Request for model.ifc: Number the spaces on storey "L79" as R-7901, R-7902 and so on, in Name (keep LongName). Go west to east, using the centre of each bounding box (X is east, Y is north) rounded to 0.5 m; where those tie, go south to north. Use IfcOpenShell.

First a look at what the model holds.

```python
import ifcopenshell
import ifcopenshell.util.element
import ifcopenshell.util.placement

model = ifcopenshell.open("model.ifc")
print(model.schema)
storey = next(s for s in model.by_type("IfcBuildingStorey") if s.Name == "L79")
spaces = [e for e in ifcopenshell.util.element.get_decomposition(storey) if e.is_a("IfcSpace")]
for e in sorted(spaces, key=lambda e: e.id()):
    origin = ifcopenshell.util.placement.get_local_placement(e.ObjectPlacement)[:3, 3]
    print(e.id(), e.Name, e.LongName, origin.round(2) + 0.0, sep=" | ")
```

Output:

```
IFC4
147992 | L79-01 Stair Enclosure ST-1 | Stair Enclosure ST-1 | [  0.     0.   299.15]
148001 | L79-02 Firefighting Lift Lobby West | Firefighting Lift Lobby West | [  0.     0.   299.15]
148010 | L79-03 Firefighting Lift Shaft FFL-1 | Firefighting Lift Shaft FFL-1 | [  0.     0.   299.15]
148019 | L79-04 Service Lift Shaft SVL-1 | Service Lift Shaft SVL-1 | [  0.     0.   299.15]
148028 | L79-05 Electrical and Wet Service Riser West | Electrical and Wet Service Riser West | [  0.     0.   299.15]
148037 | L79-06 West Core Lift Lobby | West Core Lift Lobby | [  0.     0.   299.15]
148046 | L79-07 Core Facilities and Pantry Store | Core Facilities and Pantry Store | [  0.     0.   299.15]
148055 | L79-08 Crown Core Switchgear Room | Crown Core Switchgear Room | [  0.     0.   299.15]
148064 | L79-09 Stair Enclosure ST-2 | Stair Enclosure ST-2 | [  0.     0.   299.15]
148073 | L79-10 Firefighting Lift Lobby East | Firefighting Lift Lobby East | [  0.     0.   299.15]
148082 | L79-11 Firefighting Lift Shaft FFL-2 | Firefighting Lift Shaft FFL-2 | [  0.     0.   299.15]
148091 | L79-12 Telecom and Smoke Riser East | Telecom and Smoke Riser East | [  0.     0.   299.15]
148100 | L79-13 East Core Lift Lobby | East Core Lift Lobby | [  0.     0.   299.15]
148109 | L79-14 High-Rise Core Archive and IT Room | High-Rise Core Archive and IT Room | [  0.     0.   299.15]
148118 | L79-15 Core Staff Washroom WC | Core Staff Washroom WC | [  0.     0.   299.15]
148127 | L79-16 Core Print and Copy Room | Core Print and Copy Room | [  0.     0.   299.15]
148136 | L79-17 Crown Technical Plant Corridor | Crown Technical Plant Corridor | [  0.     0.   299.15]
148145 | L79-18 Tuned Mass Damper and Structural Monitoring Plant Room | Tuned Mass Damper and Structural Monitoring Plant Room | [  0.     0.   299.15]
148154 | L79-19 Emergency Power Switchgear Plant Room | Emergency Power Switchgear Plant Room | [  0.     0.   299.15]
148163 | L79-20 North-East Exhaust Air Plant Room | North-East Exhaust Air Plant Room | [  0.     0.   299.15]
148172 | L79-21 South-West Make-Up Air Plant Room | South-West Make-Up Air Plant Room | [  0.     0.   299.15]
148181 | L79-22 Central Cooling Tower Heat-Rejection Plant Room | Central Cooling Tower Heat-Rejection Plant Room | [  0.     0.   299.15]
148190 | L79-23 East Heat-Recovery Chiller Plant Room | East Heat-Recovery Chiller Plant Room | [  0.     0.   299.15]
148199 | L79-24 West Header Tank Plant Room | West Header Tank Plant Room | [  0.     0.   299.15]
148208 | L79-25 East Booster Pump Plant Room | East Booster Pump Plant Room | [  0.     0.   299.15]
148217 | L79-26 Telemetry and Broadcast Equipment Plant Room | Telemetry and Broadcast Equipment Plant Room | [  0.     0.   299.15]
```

```python
import ifcopenshell
import ifcopenshell.geom
import ifcopenshell.util.element
import ifcopenshell.util.shape

model = ifcopenshell.open("model.ifc")
settings = ifcopenshell.geom.settings()
settings.set("use-world-coords", True)


def centre(element):
    shape = ifcopenshell.geom.create_shape(settings, element)
    return ifcopenshell.util.shape.get_bbox_centroid(shape.geometry)


storey = next(s for s in model.by_type("IfcBuildingStorey") if s.Name == "L79")
spaces = [e for e in ifcopenshell.util.element.get_decomposition(storey) if e.is_a("IfcSpace")]

# Insertion points can sit at a corner or the storey origin, so sort by the geometry (in metres).
centres = {e: centre(e) for e in spaces}
spaces.sort(key=lambda e: (round(centres[e][0] / 0.5), centres[e][1]))

for i, e in enumerate(spaces, start=1):
    number = f"R-79{i:02d}"
    e.Name = number
    print(e.id(), number)

model.write("model_v2.ifc")
```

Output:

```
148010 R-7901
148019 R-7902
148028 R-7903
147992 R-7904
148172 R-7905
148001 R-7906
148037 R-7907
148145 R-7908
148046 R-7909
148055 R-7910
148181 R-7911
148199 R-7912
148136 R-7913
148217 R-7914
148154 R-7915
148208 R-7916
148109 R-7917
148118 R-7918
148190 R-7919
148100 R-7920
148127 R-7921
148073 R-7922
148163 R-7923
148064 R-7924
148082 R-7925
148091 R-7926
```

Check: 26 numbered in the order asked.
